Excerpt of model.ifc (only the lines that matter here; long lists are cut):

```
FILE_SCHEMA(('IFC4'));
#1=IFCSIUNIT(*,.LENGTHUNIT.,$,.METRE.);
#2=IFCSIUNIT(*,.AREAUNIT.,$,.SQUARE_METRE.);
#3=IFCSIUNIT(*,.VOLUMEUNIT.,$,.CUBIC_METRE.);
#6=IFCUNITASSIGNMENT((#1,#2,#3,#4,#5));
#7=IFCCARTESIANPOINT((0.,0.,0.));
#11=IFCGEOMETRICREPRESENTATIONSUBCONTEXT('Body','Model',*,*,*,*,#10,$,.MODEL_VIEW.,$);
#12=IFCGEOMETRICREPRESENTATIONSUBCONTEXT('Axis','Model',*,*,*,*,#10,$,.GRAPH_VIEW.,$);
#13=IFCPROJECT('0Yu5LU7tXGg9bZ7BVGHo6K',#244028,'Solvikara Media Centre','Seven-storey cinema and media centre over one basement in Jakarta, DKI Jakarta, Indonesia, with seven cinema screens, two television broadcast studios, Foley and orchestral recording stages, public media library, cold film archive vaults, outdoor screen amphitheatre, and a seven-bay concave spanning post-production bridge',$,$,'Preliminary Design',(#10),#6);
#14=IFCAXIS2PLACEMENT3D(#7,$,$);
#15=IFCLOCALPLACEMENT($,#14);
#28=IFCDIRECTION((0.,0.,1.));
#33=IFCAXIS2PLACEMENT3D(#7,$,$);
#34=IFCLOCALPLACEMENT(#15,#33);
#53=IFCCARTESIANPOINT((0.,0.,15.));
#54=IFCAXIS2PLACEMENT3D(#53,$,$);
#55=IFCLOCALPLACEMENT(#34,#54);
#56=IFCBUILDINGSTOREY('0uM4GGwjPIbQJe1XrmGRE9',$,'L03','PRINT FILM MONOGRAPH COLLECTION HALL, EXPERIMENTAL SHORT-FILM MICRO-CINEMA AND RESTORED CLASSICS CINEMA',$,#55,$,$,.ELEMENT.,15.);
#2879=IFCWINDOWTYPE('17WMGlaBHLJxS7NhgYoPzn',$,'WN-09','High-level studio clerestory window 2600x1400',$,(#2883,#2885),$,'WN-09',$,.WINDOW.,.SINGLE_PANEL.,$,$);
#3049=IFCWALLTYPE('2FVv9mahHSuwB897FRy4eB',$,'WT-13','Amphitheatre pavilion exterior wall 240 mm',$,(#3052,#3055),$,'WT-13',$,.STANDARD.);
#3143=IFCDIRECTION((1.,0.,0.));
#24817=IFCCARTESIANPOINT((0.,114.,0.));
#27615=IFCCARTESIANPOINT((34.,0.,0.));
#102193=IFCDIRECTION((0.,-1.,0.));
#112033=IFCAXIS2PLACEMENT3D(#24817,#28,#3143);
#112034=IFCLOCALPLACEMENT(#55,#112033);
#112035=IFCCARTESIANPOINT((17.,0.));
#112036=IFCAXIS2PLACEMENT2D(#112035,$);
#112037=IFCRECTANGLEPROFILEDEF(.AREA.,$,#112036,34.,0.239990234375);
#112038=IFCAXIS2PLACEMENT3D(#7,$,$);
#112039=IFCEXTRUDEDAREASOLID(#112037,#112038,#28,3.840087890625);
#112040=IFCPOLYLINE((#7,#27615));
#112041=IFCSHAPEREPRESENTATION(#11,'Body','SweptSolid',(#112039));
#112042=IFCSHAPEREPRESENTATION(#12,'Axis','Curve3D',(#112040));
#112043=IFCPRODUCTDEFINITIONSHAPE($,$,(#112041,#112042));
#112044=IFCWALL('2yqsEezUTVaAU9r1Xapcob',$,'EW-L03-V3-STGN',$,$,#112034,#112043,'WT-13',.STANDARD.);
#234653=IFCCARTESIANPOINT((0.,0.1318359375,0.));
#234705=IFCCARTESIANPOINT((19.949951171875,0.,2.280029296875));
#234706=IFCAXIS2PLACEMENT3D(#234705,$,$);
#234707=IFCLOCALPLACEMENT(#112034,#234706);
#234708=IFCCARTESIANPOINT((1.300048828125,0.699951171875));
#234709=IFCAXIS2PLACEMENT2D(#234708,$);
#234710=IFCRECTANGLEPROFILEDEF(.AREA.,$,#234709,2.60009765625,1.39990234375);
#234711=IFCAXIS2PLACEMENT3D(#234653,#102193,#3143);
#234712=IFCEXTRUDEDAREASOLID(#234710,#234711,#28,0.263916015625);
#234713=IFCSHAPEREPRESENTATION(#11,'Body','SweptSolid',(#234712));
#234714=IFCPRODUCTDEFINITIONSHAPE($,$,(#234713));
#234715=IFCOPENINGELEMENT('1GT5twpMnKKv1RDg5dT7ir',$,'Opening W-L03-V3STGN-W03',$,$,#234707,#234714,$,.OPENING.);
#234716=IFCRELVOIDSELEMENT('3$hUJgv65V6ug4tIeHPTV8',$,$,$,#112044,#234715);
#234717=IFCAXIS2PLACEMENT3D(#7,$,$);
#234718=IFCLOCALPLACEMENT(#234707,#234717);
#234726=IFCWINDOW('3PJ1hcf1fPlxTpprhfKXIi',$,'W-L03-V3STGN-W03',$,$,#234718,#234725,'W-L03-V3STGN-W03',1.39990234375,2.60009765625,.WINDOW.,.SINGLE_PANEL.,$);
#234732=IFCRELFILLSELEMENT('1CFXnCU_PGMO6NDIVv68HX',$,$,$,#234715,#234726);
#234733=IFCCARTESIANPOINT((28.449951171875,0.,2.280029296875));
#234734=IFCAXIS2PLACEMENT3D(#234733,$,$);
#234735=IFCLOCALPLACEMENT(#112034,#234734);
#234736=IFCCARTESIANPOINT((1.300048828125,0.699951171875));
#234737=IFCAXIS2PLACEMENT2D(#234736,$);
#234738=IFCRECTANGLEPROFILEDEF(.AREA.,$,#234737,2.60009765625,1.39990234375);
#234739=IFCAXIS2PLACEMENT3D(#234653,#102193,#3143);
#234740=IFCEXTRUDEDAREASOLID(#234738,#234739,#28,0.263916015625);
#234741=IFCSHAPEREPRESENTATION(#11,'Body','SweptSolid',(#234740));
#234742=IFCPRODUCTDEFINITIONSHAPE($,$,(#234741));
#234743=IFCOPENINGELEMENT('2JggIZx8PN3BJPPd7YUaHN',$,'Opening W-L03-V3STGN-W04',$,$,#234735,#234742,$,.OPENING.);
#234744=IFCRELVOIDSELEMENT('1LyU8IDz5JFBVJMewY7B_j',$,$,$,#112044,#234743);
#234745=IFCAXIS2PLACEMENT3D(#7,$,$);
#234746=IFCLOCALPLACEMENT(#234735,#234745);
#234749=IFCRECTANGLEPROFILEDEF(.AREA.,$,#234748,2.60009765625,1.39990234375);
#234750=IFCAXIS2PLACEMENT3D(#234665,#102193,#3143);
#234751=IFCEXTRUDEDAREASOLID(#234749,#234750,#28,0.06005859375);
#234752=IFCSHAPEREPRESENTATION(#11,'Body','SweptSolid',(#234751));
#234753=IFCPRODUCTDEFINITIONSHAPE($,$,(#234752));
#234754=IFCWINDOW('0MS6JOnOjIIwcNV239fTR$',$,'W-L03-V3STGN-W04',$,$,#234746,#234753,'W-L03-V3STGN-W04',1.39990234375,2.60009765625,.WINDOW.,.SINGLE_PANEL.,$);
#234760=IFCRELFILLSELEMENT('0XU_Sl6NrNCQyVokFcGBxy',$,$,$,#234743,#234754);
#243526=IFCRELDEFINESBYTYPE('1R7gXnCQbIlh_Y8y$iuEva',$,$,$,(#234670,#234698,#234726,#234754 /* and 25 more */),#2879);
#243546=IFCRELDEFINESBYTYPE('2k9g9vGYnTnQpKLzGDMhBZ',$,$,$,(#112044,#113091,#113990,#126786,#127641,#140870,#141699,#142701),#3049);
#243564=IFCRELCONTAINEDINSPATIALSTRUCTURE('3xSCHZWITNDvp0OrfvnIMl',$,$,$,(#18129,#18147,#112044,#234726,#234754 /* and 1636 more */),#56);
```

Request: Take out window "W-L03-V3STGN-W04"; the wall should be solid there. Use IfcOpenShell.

```python
import ifcopenshell
import ifcopenshell.api.feature
import ifcopenshell.api.root
import ifcopenshell.geom
import ifcopenshell.util.shape

model = ifcopenshell.open("model.ifc")
settings = ifcopenshell.geom.settings()


def volume(element):
    """Net volume in cubic metres, openings subtracted."""
    shape = ifcopenshell.geom.create_shape(settings, element)
    return ifcopenshell.util.shape.get_volume(shape.geometry)


window = model.by_id(234754)
opening = window.FillsVoids[0].RelatingOpeningElement
wall = opening.VoidsElements[0].RelatingBuildingElement
before = volume(wall)

ifcopenshell.api.root.remove_product(model, product=window)
ifcopenshell.api.feature.remove_feature(model, feature=opening)

after = volume(wall)

print(f"wall volume {before:.3f} -> {after:.3f} m3")

model.write("model_v2.ifc")
```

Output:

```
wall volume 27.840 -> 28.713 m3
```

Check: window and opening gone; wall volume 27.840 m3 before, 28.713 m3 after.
